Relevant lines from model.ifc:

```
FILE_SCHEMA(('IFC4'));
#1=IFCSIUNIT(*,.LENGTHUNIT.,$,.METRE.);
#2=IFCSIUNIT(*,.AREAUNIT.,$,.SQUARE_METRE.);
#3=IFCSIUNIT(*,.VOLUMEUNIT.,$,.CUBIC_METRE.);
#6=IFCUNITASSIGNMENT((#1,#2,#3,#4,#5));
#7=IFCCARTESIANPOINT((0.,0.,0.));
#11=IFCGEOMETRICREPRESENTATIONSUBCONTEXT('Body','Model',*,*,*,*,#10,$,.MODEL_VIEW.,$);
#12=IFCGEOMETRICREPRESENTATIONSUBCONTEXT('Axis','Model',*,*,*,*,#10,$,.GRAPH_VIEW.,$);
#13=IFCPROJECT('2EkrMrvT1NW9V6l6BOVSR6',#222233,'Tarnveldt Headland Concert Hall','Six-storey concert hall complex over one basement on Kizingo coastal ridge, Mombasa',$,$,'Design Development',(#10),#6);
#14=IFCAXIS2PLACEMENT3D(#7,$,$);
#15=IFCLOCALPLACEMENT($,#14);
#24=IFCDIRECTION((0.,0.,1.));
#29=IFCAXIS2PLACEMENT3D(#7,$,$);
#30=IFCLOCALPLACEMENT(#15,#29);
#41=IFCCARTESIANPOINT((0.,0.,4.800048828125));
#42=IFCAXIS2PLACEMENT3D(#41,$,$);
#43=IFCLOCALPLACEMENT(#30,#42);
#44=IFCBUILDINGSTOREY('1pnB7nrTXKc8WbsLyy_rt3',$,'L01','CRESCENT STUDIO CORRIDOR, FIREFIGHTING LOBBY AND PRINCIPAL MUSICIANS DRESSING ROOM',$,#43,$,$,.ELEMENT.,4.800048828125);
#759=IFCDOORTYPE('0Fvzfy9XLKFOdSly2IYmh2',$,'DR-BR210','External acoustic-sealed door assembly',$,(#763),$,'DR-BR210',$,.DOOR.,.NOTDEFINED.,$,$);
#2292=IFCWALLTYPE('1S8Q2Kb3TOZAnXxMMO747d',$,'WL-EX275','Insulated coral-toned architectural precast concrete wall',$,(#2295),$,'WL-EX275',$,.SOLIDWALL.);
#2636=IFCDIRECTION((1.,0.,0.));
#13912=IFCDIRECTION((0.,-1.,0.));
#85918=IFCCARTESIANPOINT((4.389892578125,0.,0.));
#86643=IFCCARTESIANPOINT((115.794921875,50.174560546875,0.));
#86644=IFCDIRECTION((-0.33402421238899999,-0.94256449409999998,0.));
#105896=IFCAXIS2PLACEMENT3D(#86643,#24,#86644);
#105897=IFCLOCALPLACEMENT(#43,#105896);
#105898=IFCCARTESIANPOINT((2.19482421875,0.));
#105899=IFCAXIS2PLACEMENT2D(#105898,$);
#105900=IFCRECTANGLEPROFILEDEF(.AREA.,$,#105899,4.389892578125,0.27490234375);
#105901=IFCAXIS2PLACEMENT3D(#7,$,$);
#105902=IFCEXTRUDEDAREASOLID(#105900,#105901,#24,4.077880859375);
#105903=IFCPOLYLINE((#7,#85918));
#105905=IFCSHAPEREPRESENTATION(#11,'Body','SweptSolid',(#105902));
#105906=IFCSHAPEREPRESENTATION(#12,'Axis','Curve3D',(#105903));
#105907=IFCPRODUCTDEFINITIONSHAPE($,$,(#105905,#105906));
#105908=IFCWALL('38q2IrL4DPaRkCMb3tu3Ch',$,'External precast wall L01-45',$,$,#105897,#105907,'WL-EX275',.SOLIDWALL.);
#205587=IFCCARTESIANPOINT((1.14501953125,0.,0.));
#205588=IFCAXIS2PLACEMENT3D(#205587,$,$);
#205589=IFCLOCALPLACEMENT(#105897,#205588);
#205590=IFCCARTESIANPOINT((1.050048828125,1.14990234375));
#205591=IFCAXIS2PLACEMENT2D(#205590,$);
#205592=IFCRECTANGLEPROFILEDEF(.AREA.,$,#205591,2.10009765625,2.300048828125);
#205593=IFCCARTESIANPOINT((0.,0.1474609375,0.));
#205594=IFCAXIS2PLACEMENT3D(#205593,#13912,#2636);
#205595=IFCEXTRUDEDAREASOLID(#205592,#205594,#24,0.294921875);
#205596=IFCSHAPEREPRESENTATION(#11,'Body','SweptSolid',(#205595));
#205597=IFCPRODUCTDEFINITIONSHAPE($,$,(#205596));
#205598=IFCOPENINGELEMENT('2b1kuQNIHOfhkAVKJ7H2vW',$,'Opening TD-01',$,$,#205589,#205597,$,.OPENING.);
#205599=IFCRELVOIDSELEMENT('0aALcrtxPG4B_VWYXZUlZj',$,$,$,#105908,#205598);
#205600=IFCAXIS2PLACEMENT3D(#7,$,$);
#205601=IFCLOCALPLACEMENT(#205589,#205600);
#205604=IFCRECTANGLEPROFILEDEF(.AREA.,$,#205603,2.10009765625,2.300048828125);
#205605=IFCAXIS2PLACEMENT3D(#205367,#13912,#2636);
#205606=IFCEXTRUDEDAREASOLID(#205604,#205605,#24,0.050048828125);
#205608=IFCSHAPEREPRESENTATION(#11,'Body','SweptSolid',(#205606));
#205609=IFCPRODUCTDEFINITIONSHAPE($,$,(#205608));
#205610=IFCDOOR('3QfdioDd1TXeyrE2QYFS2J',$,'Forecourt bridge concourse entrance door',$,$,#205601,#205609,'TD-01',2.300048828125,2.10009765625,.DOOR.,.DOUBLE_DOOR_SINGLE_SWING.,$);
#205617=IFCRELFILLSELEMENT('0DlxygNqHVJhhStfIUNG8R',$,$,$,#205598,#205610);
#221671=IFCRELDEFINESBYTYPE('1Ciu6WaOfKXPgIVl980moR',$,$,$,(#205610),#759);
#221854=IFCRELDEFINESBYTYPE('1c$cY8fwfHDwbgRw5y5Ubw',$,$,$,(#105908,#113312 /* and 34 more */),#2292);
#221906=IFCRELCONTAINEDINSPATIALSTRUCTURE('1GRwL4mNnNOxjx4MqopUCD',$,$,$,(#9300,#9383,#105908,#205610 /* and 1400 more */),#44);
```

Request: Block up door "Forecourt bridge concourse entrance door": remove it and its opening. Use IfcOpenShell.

```python
import ifcopenshell
import ifcopenshell.api.feature
import ifcopenshell.api.root
import ifcopenshell.geom
import ifcopenshell.util.shape

model = ifcopenshell.open("model.ifc")
settings = ifcopenshell.geom.settings()


def volume(element):
    """Net volume in cubic metres, openings subtracted."""
    shape = ifcopenshell.geom.create_shape(settings, element)
    return ifcopenshell.util.shape.get_volume(shape.geometry)


door = model.by_guid("3QfdioDd1TXeyrE2QYFS2J")
opening = door.FillsVoids[0].RelatingOpeningElement
wall = opening.VoidsElements[0].RelatingBuildingElement
before = volume(wall)

ifcopenshell.api.root.remove_product(model, product=door)
ifcopenshell.api.feature.remove_feature(model, feature=opening)

after = volume(wall)

print(f"wall volume {before:.3f} -> {after:.3f} m3")

model.write("model_v2.ifc")
```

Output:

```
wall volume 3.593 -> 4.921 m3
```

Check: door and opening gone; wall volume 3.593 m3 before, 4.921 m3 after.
